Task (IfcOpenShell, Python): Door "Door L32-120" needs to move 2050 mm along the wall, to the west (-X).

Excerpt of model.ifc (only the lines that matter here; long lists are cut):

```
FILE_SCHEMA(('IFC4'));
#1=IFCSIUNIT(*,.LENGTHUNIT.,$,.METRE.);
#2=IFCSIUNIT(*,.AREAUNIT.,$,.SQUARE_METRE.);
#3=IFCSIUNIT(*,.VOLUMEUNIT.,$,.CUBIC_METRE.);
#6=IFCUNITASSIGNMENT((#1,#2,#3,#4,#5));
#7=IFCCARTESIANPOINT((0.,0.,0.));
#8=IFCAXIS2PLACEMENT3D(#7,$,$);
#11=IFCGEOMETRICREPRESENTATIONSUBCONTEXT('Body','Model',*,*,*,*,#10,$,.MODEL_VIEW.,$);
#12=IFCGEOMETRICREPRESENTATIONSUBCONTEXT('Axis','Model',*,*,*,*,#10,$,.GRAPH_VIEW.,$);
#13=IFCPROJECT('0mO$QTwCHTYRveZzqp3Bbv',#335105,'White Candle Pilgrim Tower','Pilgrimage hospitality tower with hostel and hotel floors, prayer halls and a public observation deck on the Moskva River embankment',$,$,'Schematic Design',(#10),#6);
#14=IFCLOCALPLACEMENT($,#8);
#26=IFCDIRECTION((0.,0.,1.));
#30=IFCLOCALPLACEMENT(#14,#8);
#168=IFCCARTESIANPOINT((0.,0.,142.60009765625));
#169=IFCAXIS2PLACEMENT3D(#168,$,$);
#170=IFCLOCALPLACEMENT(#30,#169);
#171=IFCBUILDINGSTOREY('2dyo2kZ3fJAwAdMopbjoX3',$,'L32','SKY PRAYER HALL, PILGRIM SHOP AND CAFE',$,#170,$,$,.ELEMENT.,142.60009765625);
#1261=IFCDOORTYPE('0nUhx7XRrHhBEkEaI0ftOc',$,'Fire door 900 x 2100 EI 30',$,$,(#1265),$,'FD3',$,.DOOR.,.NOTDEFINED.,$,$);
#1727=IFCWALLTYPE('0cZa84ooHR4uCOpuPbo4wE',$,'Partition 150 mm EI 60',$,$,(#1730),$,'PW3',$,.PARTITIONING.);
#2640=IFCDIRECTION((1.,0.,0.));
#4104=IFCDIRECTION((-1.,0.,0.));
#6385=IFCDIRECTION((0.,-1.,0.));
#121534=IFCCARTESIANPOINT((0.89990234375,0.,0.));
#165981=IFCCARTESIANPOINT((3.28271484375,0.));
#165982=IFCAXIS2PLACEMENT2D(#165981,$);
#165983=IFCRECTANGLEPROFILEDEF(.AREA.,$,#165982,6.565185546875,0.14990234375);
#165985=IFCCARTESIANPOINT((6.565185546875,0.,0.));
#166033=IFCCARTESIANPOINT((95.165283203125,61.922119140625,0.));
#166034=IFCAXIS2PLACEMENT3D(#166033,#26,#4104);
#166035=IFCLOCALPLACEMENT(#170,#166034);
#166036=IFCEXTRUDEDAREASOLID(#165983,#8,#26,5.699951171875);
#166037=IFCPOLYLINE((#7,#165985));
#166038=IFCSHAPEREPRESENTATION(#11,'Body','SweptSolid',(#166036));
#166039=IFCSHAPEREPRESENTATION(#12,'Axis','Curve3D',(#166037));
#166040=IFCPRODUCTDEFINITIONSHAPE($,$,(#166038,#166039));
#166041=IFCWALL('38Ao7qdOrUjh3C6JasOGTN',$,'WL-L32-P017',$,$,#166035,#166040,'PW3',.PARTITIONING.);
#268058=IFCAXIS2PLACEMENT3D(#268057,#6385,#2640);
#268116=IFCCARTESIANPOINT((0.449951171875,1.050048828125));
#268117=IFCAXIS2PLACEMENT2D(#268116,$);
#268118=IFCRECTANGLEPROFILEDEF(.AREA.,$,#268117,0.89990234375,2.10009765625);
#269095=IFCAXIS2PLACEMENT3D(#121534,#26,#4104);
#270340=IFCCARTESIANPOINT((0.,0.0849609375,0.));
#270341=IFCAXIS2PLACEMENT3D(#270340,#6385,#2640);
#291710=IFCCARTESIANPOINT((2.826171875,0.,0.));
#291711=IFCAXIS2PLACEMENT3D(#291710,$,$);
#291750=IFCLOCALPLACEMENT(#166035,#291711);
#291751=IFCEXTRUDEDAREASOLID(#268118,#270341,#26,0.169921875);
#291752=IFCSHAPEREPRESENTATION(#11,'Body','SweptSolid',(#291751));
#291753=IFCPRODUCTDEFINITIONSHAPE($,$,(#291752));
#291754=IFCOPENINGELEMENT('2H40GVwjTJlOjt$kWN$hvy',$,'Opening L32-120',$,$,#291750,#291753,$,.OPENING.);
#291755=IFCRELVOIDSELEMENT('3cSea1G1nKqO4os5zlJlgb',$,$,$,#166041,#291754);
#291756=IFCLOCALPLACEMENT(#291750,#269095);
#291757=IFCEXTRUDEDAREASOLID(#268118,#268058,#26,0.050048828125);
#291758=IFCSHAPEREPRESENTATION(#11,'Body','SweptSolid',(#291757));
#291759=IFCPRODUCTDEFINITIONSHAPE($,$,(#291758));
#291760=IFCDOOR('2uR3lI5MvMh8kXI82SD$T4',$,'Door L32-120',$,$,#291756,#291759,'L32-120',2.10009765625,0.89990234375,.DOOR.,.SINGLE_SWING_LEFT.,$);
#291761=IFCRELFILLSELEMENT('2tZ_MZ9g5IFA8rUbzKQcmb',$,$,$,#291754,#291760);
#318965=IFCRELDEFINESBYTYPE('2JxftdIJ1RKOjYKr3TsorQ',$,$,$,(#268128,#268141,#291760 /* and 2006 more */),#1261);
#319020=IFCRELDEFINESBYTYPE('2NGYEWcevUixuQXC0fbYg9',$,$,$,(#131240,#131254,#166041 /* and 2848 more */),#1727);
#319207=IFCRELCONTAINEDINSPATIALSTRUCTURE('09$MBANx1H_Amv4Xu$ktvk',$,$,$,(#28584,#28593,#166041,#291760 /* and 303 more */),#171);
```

```python
import ifcopenshell
import ifcopenshell.api.geometry
import ifcopenshell.util.placement

model = ifcopenshell.open("model.ifc")

door = model.by_guid("2uR3lI5MvMh8kXI82SD$T4")
opening = door.FillsVoids[0].RelatingOpeningElement
wall = opening.VoidsElements[0].RelatingBuildingElement

wall_matrix = ifcopenshell.util.placement.get_local_placement(wall.ObjectPlacement)
shift = wall_matrix[:3, 0] * 2.05
before = ifcopenshell.util.placement.get_local_placement(door.ObjectPlacement)[:3, 3].copy()

# The door is placed relative to its opening, so it follows when the opening moves.
matrix = ifcopenshell.util.placement.get_local_placement(opening.ObjectPlacement)
matrix[:3, 3] += shift
ifcopenshell.api.geometry.edit_object_placement(
    model, product=opening, matrix=matrix, is_si=False, should_transform_children=True
)

after = ifcopenshell.util.placement.get_local_placement(door.ObjectPlacement)[:3, 3]
print("door moved by", (after - before).round(3) + 0.0)

model.write("model_edited.ifc")
```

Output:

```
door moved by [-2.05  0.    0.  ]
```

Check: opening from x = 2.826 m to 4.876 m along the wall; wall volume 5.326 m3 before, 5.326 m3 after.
